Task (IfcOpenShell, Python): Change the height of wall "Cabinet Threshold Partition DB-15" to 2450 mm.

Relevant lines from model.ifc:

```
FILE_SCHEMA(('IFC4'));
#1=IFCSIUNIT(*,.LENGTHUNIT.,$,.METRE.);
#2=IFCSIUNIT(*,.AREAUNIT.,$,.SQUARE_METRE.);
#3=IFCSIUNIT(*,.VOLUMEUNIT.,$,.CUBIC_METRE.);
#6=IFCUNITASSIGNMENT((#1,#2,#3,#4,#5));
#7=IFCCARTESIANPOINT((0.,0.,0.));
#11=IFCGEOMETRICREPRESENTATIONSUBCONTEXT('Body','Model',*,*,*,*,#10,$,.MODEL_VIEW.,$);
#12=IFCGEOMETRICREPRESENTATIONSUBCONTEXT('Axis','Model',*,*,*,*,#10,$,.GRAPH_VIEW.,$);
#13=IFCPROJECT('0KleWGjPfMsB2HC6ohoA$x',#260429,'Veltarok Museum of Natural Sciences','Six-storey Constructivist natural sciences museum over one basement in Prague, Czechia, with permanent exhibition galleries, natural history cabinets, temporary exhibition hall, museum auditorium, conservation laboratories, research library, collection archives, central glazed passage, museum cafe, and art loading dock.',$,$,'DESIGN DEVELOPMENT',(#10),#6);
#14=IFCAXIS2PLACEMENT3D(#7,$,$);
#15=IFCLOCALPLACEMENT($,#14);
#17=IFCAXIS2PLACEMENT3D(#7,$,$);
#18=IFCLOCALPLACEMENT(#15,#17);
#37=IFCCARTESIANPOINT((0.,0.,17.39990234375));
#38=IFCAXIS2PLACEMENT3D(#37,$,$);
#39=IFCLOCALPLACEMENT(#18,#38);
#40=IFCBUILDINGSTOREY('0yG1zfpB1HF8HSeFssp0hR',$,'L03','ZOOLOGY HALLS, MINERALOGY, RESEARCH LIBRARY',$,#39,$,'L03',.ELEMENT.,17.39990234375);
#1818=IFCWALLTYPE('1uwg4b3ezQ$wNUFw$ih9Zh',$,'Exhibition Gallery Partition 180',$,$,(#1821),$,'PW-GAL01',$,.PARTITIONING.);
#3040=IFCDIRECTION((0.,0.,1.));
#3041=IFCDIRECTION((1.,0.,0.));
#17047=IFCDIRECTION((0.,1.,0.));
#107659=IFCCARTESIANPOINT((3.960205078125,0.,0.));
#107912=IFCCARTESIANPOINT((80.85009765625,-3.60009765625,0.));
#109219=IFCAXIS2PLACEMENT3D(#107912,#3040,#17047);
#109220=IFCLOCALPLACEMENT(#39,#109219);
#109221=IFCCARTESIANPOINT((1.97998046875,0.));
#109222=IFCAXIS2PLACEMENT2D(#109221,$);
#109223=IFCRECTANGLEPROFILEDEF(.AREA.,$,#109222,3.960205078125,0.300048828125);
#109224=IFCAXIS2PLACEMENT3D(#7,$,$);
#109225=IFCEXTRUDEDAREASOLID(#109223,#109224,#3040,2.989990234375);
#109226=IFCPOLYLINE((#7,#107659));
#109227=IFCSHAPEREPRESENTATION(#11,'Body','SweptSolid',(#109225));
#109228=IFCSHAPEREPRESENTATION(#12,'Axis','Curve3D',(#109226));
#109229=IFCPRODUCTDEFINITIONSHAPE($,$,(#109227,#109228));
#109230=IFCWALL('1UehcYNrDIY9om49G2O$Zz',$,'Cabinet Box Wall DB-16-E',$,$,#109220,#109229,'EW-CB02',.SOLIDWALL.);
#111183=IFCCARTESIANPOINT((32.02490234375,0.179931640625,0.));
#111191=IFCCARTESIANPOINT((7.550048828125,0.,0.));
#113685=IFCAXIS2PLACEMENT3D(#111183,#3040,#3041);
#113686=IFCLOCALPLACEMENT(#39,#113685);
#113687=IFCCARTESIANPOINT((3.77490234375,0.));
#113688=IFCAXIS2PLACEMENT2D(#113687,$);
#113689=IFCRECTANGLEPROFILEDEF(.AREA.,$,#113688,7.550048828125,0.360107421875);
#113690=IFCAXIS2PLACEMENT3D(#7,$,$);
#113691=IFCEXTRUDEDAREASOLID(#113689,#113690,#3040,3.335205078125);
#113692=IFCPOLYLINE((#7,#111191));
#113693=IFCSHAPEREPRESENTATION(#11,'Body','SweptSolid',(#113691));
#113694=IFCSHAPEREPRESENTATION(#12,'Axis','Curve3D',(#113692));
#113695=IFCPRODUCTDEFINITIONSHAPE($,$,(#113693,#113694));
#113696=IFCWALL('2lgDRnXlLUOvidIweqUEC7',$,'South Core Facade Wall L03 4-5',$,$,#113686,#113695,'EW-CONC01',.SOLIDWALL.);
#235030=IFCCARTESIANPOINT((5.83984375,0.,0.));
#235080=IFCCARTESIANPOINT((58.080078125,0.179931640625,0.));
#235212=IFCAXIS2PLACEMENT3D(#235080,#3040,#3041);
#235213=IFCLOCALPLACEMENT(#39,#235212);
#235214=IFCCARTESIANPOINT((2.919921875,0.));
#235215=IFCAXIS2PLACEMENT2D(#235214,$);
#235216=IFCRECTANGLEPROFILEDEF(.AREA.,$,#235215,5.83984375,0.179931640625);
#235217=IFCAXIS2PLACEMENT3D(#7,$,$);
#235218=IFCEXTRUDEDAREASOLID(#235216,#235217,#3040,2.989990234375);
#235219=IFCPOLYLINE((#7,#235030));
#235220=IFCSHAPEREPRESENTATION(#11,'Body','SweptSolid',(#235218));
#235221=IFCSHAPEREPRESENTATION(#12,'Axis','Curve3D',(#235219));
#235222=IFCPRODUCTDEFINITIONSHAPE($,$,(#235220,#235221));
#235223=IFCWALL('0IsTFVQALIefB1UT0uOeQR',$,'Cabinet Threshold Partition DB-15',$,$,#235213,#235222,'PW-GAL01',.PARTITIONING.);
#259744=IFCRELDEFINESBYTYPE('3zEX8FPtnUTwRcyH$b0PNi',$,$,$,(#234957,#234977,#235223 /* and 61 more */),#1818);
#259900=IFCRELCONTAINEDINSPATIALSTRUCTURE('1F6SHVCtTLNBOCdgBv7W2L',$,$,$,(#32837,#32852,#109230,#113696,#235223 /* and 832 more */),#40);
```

```python
import ifcopenshell
import ifcopenshell.geom
import ifcopenshell.util.representation
import ifcopenshell.util.shape

model = ifcopenshell.open("model.ifc")
settings = ifcopenshell.geom.settings()


def volume(element):
    """Net volume in cubic metres, openings subtracted."""
    shape = ifcopenshell.geom.create_shape(settings, element)
    return ifcopenshell.util.shape.get_volume(shape.geometry)


wall = model.by_guid("0IsTFVQALIefB1UT0uOeQR")
before = volume(wall)

body = ifcopenshell.util.representation.get_representation(wall, "Model", "Body")
solid = body.Items[0]
old_height = solid.Depth
solid.Depth = 2.45
after = volume(wall)

print(f"height {old_height:g} -> {solid.Depth:g}, volume {before:.3f} -> {after:.3f} m3")

model.write("model_v2.ifc")
```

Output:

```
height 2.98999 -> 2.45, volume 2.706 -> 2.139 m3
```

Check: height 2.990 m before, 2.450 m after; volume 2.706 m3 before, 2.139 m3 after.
